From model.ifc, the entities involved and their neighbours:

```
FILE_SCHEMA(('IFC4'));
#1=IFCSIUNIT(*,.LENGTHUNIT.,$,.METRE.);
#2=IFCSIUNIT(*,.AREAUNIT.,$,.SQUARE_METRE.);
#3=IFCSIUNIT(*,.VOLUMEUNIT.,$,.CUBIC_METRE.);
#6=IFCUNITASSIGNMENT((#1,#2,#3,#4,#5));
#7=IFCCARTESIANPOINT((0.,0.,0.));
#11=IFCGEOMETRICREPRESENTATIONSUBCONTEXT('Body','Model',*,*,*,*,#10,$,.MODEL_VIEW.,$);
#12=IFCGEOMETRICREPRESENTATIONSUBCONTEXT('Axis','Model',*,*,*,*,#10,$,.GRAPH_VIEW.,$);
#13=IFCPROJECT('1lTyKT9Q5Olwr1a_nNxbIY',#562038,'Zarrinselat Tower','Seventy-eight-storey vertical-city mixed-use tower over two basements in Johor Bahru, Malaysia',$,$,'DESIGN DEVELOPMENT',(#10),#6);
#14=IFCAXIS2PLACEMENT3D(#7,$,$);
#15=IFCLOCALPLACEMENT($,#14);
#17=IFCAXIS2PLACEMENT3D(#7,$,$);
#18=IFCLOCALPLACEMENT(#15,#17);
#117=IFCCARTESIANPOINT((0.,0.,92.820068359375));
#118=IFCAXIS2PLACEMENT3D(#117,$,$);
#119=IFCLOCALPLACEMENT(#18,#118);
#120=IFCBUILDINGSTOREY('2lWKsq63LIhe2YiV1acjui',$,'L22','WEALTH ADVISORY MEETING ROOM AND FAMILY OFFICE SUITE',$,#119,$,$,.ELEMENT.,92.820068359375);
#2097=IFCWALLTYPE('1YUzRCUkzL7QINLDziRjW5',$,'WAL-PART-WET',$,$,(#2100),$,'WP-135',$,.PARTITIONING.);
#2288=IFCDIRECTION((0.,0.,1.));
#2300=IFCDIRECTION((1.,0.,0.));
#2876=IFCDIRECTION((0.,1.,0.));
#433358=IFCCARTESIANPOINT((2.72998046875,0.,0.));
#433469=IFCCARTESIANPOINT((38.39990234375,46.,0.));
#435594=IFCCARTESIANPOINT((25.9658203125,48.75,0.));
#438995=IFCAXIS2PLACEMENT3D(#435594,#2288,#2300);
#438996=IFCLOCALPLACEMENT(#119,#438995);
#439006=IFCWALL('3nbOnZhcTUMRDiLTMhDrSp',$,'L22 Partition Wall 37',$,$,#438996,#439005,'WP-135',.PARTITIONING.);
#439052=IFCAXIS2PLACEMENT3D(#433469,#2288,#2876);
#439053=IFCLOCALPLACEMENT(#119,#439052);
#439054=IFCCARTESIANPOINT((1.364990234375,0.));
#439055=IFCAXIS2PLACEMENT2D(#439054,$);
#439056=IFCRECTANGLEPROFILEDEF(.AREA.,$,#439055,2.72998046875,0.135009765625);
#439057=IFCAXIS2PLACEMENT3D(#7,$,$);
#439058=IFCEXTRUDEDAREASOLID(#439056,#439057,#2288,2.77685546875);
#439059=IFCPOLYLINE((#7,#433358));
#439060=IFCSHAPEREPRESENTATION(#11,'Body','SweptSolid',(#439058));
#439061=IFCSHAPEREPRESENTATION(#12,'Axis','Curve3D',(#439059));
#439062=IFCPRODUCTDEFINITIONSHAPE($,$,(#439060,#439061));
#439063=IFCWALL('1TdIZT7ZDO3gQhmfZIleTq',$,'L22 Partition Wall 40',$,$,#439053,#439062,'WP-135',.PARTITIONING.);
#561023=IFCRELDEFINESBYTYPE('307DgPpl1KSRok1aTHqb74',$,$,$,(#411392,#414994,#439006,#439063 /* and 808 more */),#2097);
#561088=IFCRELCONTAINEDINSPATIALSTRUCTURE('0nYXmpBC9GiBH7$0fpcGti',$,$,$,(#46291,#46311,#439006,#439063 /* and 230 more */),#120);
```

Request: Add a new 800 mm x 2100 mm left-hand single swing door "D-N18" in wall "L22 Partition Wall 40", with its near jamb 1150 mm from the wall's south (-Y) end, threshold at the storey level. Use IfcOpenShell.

```python
import numpy as np
import ifcopenshell
import ifcopenshell.api.feature
import ifcopenshell.api.geometry
import ifcopenshell.api.root
import ifcopenshell.api.spatial
import ifcopenshell.geom
import ifcopenshell.util.element
import ifcopenshell.util.placement
import ifcopenshell.util.representation
import ifcopenshell.util.shape
import ifcopenshell.util.unit

model = ifcopenshell.open("model.ifc")
unit_scale = ifcopenshell.util.unit.calculate_unit_scale(model)
settings = ifcopenshell.geom.settings()


def volume(element):
    """Net volume in cubic metres, openings subtracted."""
    shape = ifcopenshell.geom.create_shape(settings, element)
    return ifcopenshell.util.shape.get_volume(shape.geometry)


wall = model.by_guid("1TdIZT7ZDO3gQhmfZIleTq")
storey = ifcopenshell.util.element.get_container(wall, ifc_class="IfcBuildingStorey")
context = ifcopenshell.util.representation.get_context(model, "Model", "Body", "MODEL_VIEW")
before = volume(wall)

width, height, from_end, sill = 0.8, 2.1, 1.15, 0.0  # metres

# The wall runs along its own X axis, and the end named is its -X end.
wall_shape = ifcopenshell.geom.create_shape(settings, wall)
x, y, z = ifcopenshell.util.shape.get_vertices(wall_shape.geometry).T
start = x.min() + from_end
face, thickness = float(y.min()), float(y.max() - y.min())
wall_matrix = ifcopenshell.util.placement.get_local_placement(wall.ObjectPlacement)
level = ifcopenshell.util.placement.get_local_placement(storey.ObjectPlacement)[2, 3]


def in_wall(x, y):
    """Placement at x, y metres in the wall's axes, at sill height."""
    matrix = wall_matrix.copy()
    matrix[:, 3] = wall_matrix @ np.array([x / unit_scale, y / unit_scale, 0.0, 1.0])
    matrix[2, 3] = level + sill / unit_scale
    return matrix


# Opening: a box that overshoots both wall faces by 50 mm.
opening = ifcopenshell.api.root.create_entity(model, ifc_class="IfcOpeningElement", predefined_type="OPENING")
box = ifcopenshell.api.geometry.add_wall_representation(
    model, context=context, length=width, height=height, thickness=thickness + 0.1
)
ifcopenshell.api.geometry.assign_representation(model, product=opening, representation=box)
ifcopenshell.api.geometry.edit_object_placement(model, product=opening, matrix=in_wall(start, face - 0.05), is_si=False)
ifcopenshell.api.feature.add_feature(model, feature=opening, element=wall)

door = ifcopenshell.api.root.create_entity(model, ifc_class="IfcDoor", name="D-N18", predefined_type="DOOR")
door.OverallWidth, door.OverallHeight = width / unit_scale, height / unit_scale
door.OperationType = "SINGLE_SWING_LEFT"
body = ifcopenshell.api.geometry.add_door_representation(
    model,
    context=context,
    overall_width=door.OverallWidth,
    overall_height=door.OverallHeight,
    operation_type="SINGLE_SWING_LEFT",
    lining_properties={"LiningDepth": thickness / unit_scale, "ThresholdDepth": thickness / unit_scale},
)
ifcopenshell.api.geometry.assign_representation(model, product=door, representation=body)
ifcopenshell.api.spatial.assign_container(model, products=[door], relating_structure=storey)
ifcopenshell.api.feature.add_filling(model, opening=opening, element=door)

# The lining spans the wall, so the door starts at the wall face.
ifcopenshell.api.geometry.edit_object_placement(model, product=door, matrix=in_wall(start, face), is_si=False)

after = volume(wall)

print(f"wall volume {before:.3f} -> {after:.3f} m3")

model.write("model_edited.ifc")
```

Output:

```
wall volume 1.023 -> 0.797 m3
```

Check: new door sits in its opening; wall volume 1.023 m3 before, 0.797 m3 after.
